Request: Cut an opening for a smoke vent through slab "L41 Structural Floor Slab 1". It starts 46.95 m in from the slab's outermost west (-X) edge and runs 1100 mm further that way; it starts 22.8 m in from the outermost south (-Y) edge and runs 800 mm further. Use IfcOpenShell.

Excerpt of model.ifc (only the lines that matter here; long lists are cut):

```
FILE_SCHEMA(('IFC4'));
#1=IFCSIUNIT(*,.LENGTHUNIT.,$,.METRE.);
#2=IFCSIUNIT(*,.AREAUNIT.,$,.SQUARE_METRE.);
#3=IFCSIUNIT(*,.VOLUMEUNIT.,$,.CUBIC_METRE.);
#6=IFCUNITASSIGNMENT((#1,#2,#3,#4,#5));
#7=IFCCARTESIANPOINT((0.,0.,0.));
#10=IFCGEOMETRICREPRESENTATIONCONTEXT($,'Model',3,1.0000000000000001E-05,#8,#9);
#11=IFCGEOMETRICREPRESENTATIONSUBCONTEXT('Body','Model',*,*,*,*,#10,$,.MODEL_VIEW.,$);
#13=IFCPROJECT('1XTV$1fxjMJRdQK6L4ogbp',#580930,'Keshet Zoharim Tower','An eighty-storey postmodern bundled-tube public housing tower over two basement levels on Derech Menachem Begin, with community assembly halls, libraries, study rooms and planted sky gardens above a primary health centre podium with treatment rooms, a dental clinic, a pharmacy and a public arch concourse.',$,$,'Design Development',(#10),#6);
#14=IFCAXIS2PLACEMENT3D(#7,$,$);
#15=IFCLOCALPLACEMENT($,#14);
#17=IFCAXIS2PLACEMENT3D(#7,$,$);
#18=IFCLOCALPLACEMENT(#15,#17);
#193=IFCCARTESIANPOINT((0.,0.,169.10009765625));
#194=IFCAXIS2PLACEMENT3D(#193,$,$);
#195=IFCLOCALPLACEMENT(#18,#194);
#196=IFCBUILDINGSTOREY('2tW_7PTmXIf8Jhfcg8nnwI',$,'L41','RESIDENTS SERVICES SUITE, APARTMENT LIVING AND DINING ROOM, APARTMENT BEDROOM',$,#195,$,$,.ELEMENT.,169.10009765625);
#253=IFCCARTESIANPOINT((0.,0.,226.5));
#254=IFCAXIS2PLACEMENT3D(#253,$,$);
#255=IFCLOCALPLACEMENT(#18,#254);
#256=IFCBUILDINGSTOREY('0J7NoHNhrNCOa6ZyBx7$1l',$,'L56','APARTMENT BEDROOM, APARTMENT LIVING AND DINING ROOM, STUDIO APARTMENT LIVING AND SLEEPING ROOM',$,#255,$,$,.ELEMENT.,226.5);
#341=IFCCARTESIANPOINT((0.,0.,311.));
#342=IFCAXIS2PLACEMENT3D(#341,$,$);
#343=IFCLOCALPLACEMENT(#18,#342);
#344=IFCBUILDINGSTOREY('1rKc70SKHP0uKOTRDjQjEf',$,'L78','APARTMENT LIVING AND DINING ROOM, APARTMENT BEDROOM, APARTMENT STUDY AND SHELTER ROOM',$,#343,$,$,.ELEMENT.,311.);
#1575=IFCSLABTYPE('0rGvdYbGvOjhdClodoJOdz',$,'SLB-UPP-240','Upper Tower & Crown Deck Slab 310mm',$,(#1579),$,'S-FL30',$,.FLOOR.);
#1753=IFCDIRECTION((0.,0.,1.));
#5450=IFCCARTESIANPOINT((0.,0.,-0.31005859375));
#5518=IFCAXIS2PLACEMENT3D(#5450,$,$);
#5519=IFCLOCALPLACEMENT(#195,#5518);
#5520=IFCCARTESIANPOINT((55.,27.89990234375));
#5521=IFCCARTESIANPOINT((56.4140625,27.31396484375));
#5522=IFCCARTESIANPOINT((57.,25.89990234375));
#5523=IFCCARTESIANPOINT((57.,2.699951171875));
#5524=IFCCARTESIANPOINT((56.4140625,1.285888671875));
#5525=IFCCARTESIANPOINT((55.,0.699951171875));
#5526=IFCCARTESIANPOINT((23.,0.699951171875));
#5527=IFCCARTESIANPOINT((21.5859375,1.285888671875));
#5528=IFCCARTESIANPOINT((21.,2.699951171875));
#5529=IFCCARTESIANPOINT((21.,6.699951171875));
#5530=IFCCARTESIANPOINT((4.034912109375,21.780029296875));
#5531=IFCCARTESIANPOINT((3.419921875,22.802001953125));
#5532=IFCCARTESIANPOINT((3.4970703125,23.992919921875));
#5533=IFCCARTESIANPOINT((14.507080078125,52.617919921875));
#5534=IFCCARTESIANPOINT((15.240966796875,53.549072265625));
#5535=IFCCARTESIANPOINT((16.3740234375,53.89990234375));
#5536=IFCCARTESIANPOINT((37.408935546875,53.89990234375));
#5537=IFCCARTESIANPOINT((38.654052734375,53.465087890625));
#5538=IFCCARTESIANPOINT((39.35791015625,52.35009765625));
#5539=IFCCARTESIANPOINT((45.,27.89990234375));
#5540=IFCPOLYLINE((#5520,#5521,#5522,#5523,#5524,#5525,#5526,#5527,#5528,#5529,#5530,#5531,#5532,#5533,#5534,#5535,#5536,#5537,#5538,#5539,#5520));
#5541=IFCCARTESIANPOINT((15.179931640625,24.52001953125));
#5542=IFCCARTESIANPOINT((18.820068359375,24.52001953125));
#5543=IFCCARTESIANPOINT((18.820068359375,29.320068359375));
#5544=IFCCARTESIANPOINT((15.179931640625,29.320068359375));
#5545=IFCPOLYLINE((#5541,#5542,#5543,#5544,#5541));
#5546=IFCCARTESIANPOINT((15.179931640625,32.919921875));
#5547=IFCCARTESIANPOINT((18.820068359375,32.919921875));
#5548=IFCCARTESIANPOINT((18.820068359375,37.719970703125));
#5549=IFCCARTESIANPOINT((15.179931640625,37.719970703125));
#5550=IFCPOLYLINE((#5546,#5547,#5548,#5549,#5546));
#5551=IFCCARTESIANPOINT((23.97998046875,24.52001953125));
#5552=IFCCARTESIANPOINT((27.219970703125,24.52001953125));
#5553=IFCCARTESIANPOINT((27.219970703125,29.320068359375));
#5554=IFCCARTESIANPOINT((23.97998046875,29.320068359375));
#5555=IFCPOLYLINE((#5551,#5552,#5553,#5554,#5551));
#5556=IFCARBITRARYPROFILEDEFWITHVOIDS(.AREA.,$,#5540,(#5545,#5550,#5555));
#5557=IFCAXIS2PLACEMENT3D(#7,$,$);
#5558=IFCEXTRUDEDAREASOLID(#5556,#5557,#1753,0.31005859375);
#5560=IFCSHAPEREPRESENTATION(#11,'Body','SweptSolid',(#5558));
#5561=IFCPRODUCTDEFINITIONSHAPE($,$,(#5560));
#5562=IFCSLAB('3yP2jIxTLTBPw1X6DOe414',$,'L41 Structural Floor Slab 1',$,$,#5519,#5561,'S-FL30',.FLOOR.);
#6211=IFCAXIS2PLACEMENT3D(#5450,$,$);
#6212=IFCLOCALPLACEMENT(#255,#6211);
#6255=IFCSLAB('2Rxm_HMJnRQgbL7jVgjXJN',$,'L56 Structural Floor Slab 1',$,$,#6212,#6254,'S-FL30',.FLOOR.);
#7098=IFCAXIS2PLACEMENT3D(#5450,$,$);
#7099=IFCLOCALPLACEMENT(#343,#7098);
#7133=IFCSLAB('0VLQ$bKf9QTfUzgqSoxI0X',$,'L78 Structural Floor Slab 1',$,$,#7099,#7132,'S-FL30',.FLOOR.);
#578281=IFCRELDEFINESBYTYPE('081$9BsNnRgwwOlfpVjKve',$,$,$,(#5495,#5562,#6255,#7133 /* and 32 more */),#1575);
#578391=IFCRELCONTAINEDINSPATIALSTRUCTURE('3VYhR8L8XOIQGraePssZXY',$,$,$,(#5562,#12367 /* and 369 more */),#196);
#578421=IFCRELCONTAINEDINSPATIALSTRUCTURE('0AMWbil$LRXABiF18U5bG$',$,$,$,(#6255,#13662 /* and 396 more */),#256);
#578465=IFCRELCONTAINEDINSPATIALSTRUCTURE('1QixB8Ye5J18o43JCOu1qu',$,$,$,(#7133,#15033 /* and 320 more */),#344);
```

```python
import numpy as np
import ifcopenshell
import ifcopenshell.api.feature
import ifcopenshell.api.geometry
import ifcopenshell.api.root
import ifcopenshell.geom
import ifcopenshell.util.placement
import ifcopenshell.util.representation
import ifcopenshell.util.shape
import ifcopenshell.util.unit

model = ifcopenshell.open("model.ifc")
unit_scale = ifcopenshell.util.unit.calculate_unit_scale(model)
settings = ifcopenshell.geom.settings()


def volume(element):
    """Net volume in cubic metres, openings subtracted."""
    shape = ifcopenshell.geom.create_shape(settings, element)
    return ifcopenshell.util.shape.get_volume(shape.geometry)


slab = model.by_id(5562)
before = volume(slab)

# Extent in the slab's own axes, in metres. The edges named are its -X and -Y sides.
slab_shape = ifcopenshell.geom.create_shape(settings, slab)
vertices = ifcopenshell.util.shape.get_vertices(slab_shape.geometry)
x_min, y_min, bottom = vertices.min(axis=0)
top = vertices[:, 2].max()

opening = ifcopenshell.api.root.create_entity(model, ifc_class="IfcOpeningElement", name="Smoke vent opening", predefined_type="OPENING")
context = ifcopenshell.util.representation.get_context(model, "Model", "Body", "MODEL_VIEW")
width, depth = 1.1, 0.8
outline = [(0.0, 0.0), (width, 0.0), (width, depth), (0.0, depth), (0.0, 0.0)]
# Overshoot both faces by 50 mm so the cut is clean.
shape = ifcopenshell.api.geometry.add_slab_representation(
    model, context=context, depth=top - bottom + 0.1, polyline=outline
)
ifcopenshell.api.geometry.assign_representation(model, product=opening, representation=shape)

matrix = ifcopenshell.util.placement.get_local_placement(slab.ObjectPlacement)
matrix[:, 3] = matrix @ np.append(np.array([x_min + 46.95, y_min + 22.8, bottom - 0.05]) / unit_scale, 1.0)
ifcopenshell.api.geometry.edit_object_placement(model, product=opening, matrix=matrix, is_si=False)
ifcopenshell.api.feature.add_feature(model, feature=opening, element=slab)

after = volume(slab)

print(f"slab volume {before:.3f} -> {after:.3f} m3")

model.write("model_v2.ifc")
```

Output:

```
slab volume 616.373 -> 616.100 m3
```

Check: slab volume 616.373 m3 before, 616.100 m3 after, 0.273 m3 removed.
